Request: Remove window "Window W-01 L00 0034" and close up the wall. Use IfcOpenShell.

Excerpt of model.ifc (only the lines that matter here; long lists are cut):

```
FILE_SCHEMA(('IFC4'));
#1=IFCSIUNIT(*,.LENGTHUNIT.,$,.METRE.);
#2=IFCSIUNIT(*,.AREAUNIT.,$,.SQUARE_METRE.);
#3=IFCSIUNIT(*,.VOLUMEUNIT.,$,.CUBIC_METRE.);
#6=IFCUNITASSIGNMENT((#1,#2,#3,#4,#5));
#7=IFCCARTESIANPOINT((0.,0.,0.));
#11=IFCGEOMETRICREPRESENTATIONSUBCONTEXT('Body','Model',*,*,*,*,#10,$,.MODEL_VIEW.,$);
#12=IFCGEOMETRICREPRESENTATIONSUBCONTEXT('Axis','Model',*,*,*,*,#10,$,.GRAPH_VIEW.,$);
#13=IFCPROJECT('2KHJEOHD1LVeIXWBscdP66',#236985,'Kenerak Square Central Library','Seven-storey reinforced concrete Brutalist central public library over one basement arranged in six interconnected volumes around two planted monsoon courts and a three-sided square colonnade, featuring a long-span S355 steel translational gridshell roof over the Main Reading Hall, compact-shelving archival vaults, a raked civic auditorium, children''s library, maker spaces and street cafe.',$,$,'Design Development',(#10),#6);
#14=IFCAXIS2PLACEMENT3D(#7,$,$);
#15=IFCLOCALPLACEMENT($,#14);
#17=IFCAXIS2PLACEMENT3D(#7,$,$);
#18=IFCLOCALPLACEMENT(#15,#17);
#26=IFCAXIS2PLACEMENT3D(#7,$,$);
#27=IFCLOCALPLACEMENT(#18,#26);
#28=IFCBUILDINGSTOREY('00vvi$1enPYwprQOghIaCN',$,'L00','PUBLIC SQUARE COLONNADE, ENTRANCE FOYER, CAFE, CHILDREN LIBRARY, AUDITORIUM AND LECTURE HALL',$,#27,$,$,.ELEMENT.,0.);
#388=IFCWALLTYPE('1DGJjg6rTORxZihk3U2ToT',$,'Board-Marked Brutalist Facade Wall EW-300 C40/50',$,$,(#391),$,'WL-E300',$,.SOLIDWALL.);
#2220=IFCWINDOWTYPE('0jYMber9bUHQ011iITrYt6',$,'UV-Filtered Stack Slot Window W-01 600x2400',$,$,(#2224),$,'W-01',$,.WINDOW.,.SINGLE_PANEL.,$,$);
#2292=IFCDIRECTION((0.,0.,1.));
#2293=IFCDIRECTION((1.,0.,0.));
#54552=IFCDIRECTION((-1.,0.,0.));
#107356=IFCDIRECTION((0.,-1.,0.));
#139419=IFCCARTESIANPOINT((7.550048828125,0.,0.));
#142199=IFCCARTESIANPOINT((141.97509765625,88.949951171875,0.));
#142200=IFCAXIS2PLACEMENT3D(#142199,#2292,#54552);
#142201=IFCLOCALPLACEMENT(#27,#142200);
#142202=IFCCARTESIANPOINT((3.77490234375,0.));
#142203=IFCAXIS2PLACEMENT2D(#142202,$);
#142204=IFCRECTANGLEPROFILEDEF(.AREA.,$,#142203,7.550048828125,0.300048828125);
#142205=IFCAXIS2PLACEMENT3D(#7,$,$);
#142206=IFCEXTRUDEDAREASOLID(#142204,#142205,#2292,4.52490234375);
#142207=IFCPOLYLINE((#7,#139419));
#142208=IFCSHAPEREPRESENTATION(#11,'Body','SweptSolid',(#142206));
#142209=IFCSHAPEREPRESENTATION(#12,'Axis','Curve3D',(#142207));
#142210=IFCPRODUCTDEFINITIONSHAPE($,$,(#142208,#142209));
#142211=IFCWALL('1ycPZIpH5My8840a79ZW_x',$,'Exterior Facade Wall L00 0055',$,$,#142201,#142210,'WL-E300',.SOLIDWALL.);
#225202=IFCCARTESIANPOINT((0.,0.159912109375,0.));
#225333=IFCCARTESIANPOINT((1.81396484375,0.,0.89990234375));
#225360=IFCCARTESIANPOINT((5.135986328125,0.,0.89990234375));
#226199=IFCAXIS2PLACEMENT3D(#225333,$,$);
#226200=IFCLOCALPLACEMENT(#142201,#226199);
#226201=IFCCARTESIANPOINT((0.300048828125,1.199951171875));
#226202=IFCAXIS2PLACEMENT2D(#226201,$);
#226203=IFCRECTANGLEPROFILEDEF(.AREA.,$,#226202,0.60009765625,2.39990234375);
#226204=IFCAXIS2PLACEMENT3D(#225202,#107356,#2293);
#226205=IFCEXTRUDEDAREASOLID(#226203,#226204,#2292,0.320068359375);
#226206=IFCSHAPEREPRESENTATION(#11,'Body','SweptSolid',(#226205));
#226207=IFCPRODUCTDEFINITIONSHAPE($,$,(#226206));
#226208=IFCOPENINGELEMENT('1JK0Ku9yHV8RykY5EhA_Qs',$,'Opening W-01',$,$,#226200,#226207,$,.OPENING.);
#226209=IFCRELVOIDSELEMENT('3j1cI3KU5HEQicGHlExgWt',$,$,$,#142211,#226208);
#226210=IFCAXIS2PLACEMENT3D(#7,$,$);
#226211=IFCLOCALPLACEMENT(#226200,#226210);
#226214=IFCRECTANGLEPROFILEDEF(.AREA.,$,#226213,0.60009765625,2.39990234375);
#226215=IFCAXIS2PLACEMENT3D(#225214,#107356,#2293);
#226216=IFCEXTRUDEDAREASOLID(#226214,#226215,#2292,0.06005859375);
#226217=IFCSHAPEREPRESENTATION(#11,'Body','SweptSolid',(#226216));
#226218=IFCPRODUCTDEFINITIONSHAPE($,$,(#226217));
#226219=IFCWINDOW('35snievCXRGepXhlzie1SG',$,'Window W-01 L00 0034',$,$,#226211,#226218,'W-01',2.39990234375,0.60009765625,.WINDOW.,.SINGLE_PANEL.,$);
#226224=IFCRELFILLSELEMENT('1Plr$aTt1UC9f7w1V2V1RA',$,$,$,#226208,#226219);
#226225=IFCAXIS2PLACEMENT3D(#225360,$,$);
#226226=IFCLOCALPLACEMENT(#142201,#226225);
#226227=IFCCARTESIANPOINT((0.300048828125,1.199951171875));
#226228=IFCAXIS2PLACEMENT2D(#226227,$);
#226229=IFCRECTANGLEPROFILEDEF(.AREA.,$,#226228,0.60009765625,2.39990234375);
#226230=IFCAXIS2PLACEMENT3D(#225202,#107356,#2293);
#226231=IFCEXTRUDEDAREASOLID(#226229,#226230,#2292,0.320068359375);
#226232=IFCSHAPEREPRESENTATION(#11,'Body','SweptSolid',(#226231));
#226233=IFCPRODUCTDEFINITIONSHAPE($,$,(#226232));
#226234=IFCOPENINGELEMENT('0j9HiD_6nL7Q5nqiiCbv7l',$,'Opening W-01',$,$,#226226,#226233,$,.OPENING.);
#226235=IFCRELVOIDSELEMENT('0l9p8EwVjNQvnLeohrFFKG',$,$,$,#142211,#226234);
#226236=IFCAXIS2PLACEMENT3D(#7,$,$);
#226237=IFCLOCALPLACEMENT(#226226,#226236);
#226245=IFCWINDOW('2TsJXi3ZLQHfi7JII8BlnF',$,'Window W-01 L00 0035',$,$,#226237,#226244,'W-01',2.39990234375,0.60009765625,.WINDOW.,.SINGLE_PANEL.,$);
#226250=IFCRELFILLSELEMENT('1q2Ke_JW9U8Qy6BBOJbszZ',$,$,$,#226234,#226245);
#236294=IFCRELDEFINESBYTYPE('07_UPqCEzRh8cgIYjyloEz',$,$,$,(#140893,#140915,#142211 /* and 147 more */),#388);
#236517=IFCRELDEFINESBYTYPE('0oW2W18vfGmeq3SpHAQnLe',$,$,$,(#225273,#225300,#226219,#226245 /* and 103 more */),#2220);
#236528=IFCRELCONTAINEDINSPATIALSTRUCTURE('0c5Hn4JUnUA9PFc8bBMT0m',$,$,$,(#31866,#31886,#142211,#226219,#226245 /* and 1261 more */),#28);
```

```python
import ifcopenshell
import ifcopenshell.api.feature
import ifcopenshell.api.root
import ifcopenshell.geom
import ifcopenshell.util.shape

model = ifcopenshell.open("model.ifc")
settings = ifcopenshell.geom.settings()


def volume(element):
    """Net volume in cubic metres, openings subtracted."""
    shape = ifcopenshell.geom.create_shape(settings, element)
    return ifcopenshell.util.shape.get_volume(shape.geometry)


window = model.by_guid("35snievCXRGepXhlzie1SG")
opening = window.FillsVoids[0].RelatingOpeningElement
wall = opening.VoidsElements[0].RelatingBuildingElement
before = volume(wall)

ifcopenshell.api.root.remove_product(model, product=window)
ifcopenshell.api.feature.remove_feature(model, feature=opening)

after = volume(wall)

print(f"wall volume {before:.3f} -> {after:.3f} m3")

model.write("model_updated.ifc")
```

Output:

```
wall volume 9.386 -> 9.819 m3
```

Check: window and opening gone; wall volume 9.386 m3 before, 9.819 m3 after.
